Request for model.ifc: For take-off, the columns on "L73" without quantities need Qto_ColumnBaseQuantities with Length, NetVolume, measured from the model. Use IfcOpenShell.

First a look at what the model holds.

```python
import ifcopenshell
import ifcopenshell.util.element
import ifcopenshell.util.unit

model = ifcopenshell.open("model.ifc")
print(model.schema)
for unit_type in ("LENGTHUNIT", "AREAUNIT", "VOLUMEUNIT"):
    print(unit_type, ifcopenshell.util.unit.calculate_unit_scale(model, unit_type))
storey = next(s for s in model.by_type("IfcBuildingStorey") if s.Name == "L73")
columns = [e for e in ifcopenshell.util.element.get_decomposition(storey) if e.is_a("IfcColumn")]
for e in sorted(columns, key=lambda e: e.id()):
    print(e.id(), e.is_a(), e.Name, list(ifcopenshell.util.element.get_psets(e, qtos_only=True)), sep=" | ")
```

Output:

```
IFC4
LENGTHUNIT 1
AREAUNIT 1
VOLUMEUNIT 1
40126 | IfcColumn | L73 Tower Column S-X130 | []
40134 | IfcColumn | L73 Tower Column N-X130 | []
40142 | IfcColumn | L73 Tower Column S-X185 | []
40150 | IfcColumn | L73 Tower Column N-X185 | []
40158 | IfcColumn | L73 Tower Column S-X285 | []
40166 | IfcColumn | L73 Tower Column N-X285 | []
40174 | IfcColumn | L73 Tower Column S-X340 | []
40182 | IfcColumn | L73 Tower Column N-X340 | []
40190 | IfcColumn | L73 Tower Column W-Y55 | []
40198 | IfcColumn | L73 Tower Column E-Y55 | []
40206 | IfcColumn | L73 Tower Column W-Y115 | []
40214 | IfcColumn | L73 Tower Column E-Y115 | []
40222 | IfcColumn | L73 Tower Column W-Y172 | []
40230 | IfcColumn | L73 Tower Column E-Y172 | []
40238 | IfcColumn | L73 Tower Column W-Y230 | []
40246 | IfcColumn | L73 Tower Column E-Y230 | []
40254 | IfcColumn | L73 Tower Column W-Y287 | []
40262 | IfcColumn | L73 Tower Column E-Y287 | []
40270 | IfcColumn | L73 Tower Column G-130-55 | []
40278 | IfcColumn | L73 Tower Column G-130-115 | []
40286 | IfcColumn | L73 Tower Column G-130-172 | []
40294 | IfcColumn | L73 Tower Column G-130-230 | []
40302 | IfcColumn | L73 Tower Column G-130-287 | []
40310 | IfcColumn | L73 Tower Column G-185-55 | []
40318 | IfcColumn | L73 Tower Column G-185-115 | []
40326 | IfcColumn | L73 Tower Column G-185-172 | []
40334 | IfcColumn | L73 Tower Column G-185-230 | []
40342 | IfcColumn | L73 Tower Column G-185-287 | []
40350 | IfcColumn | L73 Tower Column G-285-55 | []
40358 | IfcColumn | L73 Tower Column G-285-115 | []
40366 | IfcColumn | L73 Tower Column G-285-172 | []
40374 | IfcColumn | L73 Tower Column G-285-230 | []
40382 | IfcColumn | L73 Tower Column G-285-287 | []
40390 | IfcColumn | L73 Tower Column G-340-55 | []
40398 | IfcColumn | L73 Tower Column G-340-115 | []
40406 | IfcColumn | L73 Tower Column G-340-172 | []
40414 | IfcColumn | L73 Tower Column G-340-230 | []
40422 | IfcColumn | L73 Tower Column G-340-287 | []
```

```python
import ifcopenshell
import ifcopenshell.api.pset
import ifcopenshell.geom
import ifcopenshell.util.element
import ifcopenshell.util.shape
import ifcopenshell.util.unit

model = ifcopenshell.open("model.ifc")
unit_scale = ifcopenshell.util.unit.calculate_unit_scale(model)
volume_scale = ifcopenshell.util.unit.calculate_unit_scale(model, "VOLUMEUNIT")
settings = ifcopenshell.geom.settings()

storey = next(s for s in model.by_type("IfcBuildingStorey") if s.Name == "L73")
columns = [e for e in ifcopenshell.util.element.get_decomposition(storey) if e.is_a("IfcColumn")]

for e in sorted(columns, key=lambda e: e.id()):
    if ifcopenshell.util.element.get_psets(e, qtos_only=True, should_inherit=False):
        continue
    # Geometry comes back in metres, in the element's own axes.
    shape = ifcopenshell.geom.create_shape(settings, e)
    values = {
        "Length": ifcopenshell.util.shape.get_z(shape.geometry) / unit_scale,
        "NetVolume": ifcopenshell.util.shape.get_volume(shape.geometry) / volume_scale,
    }
    qto = ifcopenshell.api.pset.add_qto(model, product=e, name="Qto_ColumnBaseQuantities")
    ifcopenshell.api.pset.edit_qto(model, qto=qto, properties=values)
    print(e.id(), {k: round(v, 3) for k, v in values.items()})

model.write("model_v2.ifc")
```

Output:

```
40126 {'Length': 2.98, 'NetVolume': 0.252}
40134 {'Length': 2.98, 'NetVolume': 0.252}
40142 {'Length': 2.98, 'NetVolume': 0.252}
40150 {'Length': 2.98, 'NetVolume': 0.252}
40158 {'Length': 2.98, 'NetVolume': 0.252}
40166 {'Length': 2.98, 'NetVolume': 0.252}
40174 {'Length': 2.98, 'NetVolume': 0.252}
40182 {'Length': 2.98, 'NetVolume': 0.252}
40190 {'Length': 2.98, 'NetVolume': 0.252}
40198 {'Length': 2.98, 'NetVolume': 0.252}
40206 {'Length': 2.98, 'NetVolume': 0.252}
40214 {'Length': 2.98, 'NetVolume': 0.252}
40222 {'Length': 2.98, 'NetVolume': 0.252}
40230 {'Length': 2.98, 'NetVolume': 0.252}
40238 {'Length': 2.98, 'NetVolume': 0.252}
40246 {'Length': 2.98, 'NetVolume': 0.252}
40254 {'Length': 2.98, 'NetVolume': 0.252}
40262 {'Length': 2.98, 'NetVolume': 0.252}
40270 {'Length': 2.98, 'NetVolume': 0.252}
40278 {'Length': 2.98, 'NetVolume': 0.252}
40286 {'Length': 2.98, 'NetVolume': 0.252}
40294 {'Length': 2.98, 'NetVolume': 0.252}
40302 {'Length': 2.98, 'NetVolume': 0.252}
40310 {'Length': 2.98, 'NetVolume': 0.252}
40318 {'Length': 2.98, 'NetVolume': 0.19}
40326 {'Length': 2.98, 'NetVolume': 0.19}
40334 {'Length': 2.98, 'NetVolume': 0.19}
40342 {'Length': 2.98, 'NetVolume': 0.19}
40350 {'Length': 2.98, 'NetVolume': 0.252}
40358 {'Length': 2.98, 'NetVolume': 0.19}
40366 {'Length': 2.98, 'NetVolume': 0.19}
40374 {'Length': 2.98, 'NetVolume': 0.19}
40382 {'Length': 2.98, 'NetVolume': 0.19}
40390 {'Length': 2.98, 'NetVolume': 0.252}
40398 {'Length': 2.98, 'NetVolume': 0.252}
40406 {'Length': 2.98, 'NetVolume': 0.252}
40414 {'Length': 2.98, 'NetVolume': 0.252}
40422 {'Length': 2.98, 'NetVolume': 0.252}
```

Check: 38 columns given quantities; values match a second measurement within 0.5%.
